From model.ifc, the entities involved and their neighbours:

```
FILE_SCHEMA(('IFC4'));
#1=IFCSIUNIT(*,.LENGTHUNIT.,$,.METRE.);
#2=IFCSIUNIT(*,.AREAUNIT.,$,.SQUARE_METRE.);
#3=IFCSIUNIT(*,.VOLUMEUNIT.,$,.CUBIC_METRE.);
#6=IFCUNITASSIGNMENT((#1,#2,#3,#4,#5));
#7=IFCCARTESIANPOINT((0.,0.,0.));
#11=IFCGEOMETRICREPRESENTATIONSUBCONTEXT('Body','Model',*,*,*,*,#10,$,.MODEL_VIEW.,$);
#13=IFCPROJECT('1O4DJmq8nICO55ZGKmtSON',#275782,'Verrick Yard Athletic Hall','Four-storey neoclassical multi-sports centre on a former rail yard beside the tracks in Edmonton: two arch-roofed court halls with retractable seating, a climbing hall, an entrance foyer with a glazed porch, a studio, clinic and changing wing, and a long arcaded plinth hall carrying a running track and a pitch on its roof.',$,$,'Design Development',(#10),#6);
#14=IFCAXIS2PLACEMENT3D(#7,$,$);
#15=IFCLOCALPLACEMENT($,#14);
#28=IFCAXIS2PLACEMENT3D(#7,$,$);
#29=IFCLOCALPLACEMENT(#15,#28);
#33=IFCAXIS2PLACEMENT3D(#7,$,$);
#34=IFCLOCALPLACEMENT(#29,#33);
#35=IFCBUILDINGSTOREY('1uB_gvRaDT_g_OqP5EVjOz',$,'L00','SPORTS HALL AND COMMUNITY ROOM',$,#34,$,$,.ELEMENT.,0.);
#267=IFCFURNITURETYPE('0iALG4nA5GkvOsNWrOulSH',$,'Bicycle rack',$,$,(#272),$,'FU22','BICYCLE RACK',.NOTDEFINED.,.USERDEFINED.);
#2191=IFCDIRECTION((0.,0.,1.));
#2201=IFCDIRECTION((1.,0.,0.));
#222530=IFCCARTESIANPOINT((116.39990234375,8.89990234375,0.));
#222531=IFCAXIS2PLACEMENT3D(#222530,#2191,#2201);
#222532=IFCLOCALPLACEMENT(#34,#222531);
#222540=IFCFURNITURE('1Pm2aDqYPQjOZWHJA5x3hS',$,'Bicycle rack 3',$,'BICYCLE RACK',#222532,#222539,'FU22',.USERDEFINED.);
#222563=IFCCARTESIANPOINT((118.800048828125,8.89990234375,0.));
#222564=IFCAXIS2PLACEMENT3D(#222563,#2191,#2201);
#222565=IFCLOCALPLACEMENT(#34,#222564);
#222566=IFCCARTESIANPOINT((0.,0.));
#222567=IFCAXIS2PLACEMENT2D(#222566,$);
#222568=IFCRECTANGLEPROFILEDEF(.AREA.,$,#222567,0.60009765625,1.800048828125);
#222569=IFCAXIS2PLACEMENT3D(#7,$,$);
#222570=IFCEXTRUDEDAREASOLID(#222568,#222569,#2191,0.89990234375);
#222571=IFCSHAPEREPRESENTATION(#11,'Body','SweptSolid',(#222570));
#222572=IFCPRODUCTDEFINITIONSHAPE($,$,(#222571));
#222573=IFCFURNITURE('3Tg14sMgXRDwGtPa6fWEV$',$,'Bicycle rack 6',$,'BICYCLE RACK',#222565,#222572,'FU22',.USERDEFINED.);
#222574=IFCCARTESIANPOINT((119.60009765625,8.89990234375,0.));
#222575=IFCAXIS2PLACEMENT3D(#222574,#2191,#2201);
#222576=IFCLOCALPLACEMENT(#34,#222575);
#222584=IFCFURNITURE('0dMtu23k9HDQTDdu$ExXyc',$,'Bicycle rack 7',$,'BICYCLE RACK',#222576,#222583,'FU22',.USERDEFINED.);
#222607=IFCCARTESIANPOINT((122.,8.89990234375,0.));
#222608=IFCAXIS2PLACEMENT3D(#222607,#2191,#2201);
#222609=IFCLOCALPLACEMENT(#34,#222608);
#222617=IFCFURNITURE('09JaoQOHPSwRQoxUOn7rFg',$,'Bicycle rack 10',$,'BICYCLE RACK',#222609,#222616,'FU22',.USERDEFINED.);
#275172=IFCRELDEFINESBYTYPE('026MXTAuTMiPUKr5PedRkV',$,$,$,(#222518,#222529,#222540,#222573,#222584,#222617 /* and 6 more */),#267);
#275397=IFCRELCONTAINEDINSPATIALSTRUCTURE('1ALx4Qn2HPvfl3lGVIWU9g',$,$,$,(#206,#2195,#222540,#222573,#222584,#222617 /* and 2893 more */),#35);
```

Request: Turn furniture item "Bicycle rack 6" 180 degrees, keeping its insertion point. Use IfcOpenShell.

```python
import ifcopenshell
import ifcopenshell.api.geometry
import ifcopenshell.util.placement

model = ifcopenshell.open("model.ifc")

item = model.by_guid("3Tg14sMgXRDwGtPa6fWEV$")
matrix = ifcopenshell.util.placement.get_local_placement(item.ObjectPlacement)
matrix = matrix @ ifcopenshell.util.placement.rotation(180, "Z")
ifcopenshell.api.geometry.edit_object_placement(model, product=item, matrix=matrix, is_si=False)

print(ifcopenshell.util.placement.get_local_placement(item.ObjectPlacement).round(3) + 0.0)

model.write("model-out.ifc")
```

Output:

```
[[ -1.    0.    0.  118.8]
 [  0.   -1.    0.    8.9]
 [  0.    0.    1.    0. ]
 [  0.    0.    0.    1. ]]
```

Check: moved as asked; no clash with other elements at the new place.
